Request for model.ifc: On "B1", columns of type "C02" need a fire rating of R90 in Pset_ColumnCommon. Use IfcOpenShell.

First a look at what the model holds.

```python
import ifcopenshell
import ifcopenshell.util.element

model = ifcopenshell.open("model.ifc")
print(model.schema)
storey = next(s for s in model.by_type("IfcBuildingStorey") if s.Name == "B1")
columns = [e for e in ifcopenshell.util.element.get_decomposition(storey) if e.is_a("IfcColumn")]
seen = {}
for e in columns:
    element_type = ifcopenshell.util.element.get_type(e)
    key = (element_type.Name if element_type != e and element_type else None, ifcopenshell.util.element.get_pset(e, "Pset_ColumnCommon", "FireRating"))
    seen[key] = seen.get(key, 0) + 1
for (name, value), count in sorted(seen.items(), key=str):
    print(count, "x", name, "|", value)
```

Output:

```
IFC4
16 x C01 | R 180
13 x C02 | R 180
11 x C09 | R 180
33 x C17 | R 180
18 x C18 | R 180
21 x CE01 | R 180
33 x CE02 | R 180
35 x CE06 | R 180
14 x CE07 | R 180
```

```python
import ifcopenshell
import ifcopenshell.api.pset
import ifcopenshell.util.element

model = ifcopenshell.open("model.ifc")

storey = next(s for s in model.by_type("IfcBuildingStorey") if s.Name == "B1")
columns = [e for e in ifcopenshell.util.element.get_decomposition(storey) if e.is_a("IfcColumn")]

count = 0
for e in columns:
    element_type = ifcopenshell.util.element.get_type(e)
    if element_type in (None, e) or element_type.Name != "C02":
        continue
    # add_pset returns the element's existing set when there is one.
    pset = ifcopenshell.api.pset.add_pset(model, product=e, name="Pset_ColumnCommon")
    ifcopenshell.api.pset.edit_pset(model, pset=pset, properties={"FireRating": "R90"})
    count += 1

print(count, "columns updated")

model.write("model_edited.ifc")
```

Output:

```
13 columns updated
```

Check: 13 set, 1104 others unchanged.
